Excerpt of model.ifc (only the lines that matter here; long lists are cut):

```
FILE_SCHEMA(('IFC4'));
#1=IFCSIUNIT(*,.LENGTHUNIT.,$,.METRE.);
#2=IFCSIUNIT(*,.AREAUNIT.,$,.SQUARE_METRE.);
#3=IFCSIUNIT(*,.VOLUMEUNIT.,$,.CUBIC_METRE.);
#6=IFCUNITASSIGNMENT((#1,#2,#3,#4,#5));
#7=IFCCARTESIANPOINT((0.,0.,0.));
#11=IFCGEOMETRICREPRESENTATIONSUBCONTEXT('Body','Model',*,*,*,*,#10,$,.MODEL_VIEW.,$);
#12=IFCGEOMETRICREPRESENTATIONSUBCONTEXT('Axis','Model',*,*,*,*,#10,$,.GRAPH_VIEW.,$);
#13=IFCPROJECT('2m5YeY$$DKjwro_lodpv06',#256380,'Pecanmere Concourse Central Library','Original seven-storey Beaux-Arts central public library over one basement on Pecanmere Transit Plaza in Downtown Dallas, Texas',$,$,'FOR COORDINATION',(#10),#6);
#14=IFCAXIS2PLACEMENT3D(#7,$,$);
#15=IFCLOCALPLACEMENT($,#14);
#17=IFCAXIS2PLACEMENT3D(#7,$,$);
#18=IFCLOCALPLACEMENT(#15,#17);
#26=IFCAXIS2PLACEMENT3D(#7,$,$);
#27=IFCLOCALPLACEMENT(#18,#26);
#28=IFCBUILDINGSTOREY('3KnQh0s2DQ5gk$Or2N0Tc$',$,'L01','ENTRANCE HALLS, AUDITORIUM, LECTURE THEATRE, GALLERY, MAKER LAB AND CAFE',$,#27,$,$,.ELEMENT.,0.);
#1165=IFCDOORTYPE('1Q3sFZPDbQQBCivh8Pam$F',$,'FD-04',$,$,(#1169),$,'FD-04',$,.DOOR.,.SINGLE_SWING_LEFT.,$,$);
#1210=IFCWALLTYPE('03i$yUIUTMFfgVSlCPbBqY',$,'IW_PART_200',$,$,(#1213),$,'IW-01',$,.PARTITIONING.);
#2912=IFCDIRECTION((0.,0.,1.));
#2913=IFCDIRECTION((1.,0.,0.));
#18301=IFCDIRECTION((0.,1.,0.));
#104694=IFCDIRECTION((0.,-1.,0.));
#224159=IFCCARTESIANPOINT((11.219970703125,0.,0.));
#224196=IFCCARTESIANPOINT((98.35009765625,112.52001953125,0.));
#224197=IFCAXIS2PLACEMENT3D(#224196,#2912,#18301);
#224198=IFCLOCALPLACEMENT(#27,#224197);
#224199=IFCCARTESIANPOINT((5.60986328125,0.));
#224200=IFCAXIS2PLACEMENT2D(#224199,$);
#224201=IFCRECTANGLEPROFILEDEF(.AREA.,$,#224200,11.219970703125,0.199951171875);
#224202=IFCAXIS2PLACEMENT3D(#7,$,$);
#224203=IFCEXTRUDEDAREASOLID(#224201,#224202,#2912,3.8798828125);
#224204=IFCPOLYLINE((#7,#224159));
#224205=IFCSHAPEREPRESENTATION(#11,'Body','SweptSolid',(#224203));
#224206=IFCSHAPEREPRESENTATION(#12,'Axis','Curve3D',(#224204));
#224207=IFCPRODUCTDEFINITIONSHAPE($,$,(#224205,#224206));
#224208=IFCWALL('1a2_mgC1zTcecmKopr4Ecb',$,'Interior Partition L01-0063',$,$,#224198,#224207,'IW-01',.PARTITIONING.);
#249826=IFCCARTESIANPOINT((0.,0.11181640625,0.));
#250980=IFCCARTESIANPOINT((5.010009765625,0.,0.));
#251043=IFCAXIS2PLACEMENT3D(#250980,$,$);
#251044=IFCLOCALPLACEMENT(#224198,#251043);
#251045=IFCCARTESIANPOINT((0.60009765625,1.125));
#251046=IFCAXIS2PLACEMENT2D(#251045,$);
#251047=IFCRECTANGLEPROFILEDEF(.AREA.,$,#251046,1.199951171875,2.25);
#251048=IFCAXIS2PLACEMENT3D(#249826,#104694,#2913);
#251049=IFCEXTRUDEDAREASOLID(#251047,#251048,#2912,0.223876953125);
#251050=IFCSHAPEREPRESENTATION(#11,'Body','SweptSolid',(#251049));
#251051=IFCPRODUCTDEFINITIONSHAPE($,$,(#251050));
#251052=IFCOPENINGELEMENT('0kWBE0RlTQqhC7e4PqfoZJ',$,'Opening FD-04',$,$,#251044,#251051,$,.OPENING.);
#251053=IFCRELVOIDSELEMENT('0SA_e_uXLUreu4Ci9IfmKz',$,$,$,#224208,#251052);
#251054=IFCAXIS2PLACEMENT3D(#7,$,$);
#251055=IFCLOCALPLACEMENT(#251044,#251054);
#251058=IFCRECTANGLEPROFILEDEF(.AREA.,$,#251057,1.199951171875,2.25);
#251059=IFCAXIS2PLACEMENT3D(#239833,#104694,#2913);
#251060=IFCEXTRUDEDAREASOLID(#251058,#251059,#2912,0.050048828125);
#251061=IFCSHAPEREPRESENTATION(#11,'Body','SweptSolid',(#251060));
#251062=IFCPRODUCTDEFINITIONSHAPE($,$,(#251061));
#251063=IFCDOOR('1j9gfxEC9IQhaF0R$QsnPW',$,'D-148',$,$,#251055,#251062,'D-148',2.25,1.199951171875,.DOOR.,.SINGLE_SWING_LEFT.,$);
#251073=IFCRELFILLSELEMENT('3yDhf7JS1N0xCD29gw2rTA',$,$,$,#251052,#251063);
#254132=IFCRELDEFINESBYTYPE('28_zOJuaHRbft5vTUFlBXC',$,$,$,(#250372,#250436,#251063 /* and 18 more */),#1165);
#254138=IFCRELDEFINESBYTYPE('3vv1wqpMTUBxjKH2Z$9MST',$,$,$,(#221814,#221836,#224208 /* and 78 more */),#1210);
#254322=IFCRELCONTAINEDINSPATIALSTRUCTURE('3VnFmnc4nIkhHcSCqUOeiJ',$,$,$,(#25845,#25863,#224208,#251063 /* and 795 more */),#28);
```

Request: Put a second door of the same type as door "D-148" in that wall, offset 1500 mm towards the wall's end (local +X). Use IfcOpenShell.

```python
import ifcopenshell
import ifcopenshell.api.feature
import ifcopenshell.api.geometry
import ifcopenshell.api.root
import ifcopenshell.geom
import ifcopenshell.util.element
import ifcopenshell.util.placement
import ifcopenshell.util.shape
import ifcopenshell.util.unit

model = ifcopenshell.open("model.ifc")
unit_scale = ifcopenshell.util.unit.calculate_unit_scale(model)
settings = ifcopenshell.geom.settings()


def volume(element):
    """Net volume in cubic metres, openings subtracted."""
    shape = ifcopenshell.geom.create_shape(settings, element)
    return ifcopenshell.util.shape.get_volume(shape.geometry)


door = model.by_guid("1j9gfxEC9IQhaF0R$QsnPW")
opening = door.FillsVoids[0].RelatingOpeningElement
wall = opening.VoidsElements[0].RelatingBuildingElement
before = volume(wall)
shift = ifcopenshell.util.placement.get_local_placement(wall.ObjectPlacement)[:3, 0] * 1.5 / unit_scale

# copy_class copies the void relationship, type, container and properties, but no geometry.
new_opening = ifcopenshell.api.root.copy_class(model, product=opening)
new_opening.Representation = ifcopenshell.util.element.copy_deep(
    model, opening.Representation, exclude=["IfcGeometricRepresentationContext", "IfcRepresentationMap"]
)
new_door = ifcopenshell.api.root.copy_class(model, product=door)
new_door.Representation = ifcopenshell.util.element.copy_deep(
    model, door.Representation, exclude=["IfcGeometricRepresentationContext", "IfcRepresentationMap"]
)
new_door.Tag = None
ifcopenshell.api.feature.add_filling(model, opening=new_opening, element=new_door)

for old, new in ((opening, new_opening), (door, new_door)):
    matrix = ifcopenshell.util.placement.get_local_placement(old.ObjectPlacement)
    matrix[:3, 3] += shift
    ifcopenshell.api.geometry.edit_object_placement(model, product=new, matrix=matrix, is_si=False)

after = volume(wall)

print(f"wall volume {before:.3f} -> {after:.3f} m3")

model.write("model_rev.ifc")
```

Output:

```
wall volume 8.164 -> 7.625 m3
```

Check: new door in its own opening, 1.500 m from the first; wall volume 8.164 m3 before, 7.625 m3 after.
